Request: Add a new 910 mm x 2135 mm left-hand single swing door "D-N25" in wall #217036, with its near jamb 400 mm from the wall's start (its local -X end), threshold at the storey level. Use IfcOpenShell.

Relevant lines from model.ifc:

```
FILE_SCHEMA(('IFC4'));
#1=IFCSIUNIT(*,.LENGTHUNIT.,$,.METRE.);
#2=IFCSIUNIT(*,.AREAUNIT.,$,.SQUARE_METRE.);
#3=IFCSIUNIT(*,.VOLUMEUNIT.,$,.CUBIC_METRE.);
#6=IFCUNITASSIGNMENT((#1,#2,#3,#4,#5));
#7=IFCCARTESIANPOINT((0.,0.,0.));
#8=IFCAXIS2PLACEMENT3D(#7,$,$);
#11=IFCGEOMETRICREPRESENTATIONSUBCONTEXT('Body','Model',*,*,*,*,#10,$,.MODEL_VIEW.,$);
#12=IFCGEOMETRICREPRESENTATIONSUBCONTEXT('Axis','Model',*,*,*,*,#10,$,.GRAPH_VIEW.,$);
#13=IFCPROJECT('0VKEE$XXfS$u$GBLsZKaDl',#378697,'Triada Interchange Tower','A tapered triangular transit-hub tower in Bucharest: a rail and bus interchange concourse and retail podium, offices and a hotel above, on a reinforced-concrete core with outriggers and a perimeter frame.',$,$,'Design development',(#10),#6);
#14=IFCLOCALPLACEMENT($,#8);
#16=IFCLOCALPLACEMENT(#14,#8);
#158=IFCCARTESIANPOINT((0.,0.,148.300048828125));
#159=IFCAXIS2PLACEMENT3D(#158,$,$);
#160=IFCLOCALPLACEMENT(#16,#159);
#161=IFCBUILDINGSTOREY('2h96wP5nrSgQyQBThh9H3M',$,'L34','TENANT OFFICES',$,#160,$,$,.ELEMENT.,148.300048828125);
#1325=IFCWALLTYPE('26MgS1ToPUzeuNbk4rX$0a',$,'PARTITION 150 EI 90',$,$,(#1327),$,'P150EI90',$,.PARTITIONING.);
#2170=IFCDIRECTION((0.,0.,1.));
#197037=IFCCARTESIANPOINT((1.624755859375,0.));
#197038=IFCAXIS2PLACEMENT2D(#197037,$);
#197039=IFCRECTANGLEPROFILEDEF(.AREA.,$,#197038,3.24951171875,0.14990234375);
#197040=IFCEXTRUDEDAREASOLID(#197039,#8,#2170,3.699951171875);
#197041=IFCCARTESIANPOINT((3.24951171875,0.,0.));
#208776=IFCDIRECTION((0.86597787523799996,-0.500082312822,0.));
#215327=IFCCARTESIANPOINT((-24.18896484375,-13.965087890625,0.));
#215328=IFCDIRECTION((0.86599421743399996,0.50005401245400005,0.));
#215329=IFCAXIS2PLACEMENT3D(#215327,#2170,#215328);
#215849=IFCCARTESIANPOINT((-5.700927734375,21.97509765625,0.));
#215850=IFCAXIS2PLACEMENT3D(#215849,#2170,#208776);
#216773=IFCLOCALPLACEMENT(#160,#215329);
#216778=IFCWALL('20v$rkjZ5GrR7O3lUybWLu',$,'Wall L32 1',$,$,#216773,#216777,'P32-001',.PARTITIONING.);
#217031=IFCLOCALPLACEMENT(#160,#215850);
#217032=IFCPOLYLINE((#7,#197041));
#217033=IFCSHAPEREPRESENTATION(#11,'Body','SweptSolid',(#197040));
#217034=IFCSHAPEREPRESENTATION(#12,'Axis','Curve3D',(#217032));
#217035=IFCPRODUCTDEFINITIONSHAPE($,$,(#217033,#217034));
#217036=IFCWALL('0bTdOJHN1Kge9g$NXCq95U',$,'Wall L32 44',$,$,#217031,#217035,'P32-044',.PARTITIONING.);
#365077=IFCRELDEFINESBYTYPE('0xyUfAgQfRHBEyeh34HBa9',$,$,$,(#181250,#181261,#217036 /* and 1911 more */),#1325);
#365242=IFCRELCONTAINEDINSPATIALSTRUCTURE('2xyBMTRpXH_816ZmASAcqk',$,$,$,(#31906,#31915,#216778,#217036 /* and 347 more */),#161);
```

```python
import numpy as np
import ifcopenshell
import ifcopenshell.api.feature
import ifcopenshell.api.geometry
import ifcopenshell.api.root
import ifcopenshell.api.spatial
import ifcopenshell.geom
import ifcopenshell.util.element
import ifcopenshell.util.placement
import ifcopenshell.util.representation
import ifcopenshell.util.shape
import ifcopenshell.util.unit

model = ifcopenshell.open("model.ifc")
unit_scale = ifcopenshell.util.unit.calculate_unit_scale(model)
settings = ifcopenshell.geom.settings()


def volume(element):
    """Net volume in cubic metres, openings subtracted."""
    shape = ifcopenshell.geom.create_shape(settings, element)
    return ifcopenshell.util.shape.get_volume(shape.geometry)


wall = model.by_guid("0bTdOJHN1Kge9g$NXCq95U")
storey = ifcopenshell.util.element.get_container(wall, ifc_class="IfcBuildingStorey")
context = ifcopenshell.util.representation.get_context(model, "Model", "Body", "MODEL_VIEW")
before = volume(wall)

width, height, from_end, sill = 0.91, 2.135, 0.4, 0.0  # metres

# The wall runs along its own X axis, and the end named is its -X end.
wall_shape = ifcopenshell.geom.create_shape(settings, wall)
x, y, z = ifcopenshell.util.shape.get_vertices(wall_shape.geometry).T
start = x.min() + from_end
face, thickness = float(y.min()), float(y.max() - y.min())
wall_matrix = ifcopenshell.util.placement.get_local_placement(wall.ObjectPlacement)
level = ifcopenshell.util.placement.get_local_placement(storey.ObjectPlacement)[2, 3]


def in_wall(x, y):
    """Placement at x, y metres in the wall's axes, at sill height."""
    matrix = wall_matrix.copy()
    matrix[:, 3] = wall_matrix @ np.array([x / unit_scale, y / unit_scale, 0.0, 1.0])
    matrix[2, 3] = level + sill / unit_scale
    return matrix


# Opening: a box that overshoots both wall faces by 50 mm.
opening = ifcopenshell.api.root.create_entity(model, ifc_class="IfcOpeningElement", predefined_type="OPENING")
box = ifcopenshell.api.geometry.add_wall_representation(
    model, context=context, length=width, height=height, thickness=thickness + 0.1
)
ifcopenshell.api.geometry.assign_representation(model, product=opening, representation=box)
ifcopenshell.api.geometry.edit_object_placement(model, product=opening, matrix=in_wall(start, face - 0.05), is_si=False)
ifcopenshell.api.feature.add_feature(model, feature=opening, element=wall)

door = ifcopenshell.api.root.create_entity(model, ifc_class="IfcDoor", name="D-N25", predefined_type="DOOR")
door.OverallWidth, door.OverallHeight = width / unit_scale, height / unit_scale
door.OperationType = "SINGLE_SWING_LEFT"
body = ifcopenshell.api.geometry.add_door_representation(
    model,
    context=context,
    overall_width=door.OverallWidth,
    overall_height=door.OverallHeight,
    operation_type="SINGLE_SWING_LEFT",
    lining_properties={"LiningDepth": thickness / unit_scale, "ThresholdDepth": thickness / unit_scale},
)
ifcopenshell.api.geometry.assign_representation(model, product=door, representation=body)
ifcopenshell.api.spatial.assign_container(model, products=[door], relating_structure=storey)
ifcopenshell.api.feature.add_filling(model, opening=opening, element=door)

# The lining spans the wall, so the door starts at the wall face.
ifcopenshell.api.geometry.edit_object_placement(model, product=door, matrix=in_wall(start, face), is_si=False)

after = volume(wall)

print(f"wall volume {before:.3f} -> {after:.3f} m3")

model.write("model-out.ifc")
```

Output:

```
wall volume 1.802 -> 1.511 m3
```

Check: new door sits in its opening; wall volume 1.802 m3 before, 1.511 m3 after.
